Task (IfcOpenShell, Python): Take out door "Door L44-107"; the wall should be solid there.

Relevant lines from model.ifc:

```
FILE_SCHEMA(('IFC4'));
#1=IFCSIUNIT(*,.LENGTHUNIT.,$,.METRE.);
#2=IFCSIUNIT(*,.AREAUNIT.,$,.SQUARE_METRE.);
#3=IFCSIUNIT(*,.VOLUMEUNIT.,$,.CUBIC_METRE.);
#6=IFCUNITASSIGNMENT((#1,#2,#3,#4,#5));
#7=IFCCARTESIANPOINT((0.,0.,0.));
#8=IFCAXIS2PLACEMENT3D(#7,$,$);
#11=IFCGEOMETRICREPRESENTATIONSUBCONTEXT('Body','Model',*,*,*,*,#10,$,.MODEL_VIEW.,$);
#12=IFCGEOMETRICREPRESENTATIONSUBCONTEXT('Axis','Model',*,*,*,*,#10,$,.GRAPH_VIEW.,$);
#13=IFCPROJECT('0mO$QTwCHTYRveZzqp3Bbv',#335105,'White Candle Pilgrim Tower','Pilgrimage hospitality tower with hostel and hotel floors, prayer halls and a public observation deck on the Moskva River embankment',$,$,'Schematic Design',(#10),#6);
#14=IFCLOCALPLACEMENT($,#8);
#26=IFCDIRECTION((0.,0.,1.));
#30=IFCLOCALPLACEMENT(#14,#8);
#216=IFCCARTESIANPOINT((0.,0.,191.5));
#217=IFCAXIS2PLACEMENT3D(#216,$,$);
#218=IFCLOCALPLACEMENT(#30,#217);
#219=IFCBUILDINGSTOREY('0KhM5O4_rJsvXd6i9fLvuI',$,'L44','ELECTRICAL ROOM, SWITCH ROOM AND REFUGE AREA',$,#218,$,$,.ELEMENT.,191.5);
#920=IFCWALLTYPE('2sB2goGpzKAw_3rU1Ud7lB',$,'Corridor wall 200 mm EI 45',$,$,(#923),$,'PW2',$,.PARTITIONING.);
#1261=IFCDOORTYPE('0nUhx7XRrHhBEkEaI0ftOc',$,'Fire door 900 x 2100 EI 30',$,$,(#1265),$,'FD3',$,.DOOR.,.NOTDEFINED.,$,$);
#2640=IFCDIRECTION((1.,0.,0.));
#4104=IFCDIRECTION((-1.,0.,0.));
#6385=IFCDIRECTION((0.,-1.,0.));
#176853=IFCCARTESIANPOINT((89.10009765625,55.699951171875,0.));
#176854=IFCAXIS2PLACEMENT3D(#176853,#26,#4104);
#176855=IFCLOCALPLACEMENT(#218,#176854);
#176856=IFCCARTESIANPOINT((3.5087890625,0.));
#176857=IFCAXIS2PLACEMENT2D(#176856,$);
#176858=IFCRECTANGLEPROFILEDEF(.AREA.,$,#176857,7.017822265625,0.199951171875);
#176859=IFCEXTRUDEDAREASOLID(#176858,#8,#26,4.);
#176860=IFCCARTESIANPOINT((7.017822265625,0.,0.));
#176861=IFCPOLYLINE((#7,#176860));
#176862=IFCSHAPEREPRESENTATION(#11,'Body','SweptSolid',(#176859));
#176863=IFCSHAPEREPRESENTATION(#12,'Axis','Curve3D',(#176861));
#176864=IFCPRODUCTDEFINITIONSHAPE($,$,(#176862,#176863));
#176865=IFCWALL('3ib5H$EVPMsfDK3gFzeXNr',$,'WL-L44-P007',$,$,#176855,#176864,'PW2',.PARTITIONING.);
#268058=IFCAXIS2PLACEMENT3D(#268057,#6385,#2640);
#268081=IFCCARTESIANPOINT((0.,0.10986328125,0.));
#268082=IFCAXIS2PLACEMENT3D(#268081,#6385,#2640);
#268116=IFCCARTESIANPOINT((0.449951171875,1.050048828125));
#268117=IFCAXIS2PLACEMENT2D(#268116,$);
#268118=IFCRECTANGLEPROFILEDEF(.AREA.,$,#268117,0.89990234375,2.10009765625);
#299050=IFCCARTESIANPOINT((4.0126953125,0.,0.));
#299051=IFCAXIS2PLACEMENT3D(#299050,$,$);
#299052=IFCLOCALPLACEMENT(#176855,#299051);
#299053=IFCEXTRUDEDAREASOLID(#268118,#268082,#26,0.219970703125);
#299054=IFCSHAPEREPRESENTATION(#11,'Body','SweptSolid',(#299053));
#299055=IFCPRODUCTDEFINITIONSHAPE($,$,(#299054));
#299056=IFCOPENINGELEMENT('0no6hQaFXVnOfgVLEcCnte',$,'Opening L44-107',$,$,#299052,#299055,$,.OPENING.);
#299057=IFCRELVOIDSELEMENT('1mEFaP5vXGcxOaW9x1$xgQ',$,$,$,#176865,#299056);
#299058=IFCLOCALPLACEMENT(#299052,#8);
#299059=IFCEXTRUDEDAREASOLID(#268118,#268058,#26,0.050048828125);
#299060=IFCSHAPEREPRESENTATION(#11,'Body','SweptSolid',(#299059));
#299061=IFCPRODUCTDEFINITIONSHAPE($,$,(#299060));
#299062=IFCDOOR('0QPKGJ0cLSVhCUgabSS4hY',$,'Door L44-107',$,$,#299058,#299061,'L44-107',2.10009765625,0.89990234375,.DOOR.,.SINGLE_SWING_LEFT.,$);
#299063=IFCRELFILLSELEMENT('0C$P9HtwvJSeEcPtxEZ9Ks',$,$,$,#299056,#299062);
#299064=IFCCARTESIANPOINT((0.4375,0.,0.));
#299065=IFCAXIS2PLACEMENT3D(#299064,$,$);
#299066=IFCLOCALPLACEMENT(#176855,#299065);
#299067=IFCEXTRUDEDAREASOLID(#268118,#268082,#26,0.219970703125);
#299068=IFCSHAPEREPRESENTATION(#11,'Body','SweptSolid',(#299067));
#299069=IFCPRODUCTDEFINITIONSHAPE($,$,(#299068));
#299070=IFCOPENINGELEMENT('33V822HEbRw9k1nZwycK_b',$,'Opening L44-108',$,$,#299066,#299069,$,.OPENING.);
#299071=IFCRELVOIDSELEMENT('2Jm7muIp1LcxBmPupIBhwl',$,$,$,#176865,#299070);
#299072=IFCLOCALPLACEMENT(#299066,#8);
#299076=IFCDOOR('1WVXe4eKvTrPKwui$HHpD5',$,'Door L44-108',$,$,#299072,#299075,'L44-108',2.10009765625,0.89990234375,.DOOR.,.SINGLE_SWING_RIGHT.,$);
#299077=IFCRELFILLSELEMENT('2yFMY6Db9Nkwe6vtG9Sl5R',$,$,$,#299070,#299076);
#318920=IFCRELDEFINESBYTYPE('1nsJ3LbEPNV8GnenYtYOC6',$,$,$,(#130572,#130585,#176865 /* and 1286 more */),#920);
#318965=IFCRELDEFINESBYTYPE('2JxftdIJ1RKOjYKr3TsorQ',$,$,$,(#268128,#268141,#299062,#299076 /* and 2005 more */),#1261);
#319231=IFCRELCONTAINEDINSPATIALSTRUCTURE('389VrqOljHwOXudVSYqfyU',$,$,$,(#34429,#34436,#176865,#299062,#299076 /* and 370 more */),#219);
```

```python
import ifcopenshell
import ifcopenshell.api.feature
import ifcopenshell.api.root
import ifcopenshell.geom
import ifcopenshell.util.shape

model = ifcopenshell.open("model.ifc")
settings = ifcopenshell.geom.settings()


def volume(element):
    """Net volume in cubic metres, openings subtracted."""
    shape = ifcopenshell.geom.create_shape(settings, element)
    return ifcopenshell.util.shape.get_volume(shape.geometry)


door = model.by_id(299062)
opening = door.FillsVoids[0].RelatingOpeningElement
wall = opening.VoidsElements[0].RelatingBuildingElement
before = volume(wall)

ifcopenshell.api.root.remove_product(model, product=door)
ifcopenshell.api.feature.remove_feature(model, feature=opening)

after = volume(wall)

print(f"wall volume {before:.3f} -> {after:.3f} m3")

model.write("model-out.ifc")
```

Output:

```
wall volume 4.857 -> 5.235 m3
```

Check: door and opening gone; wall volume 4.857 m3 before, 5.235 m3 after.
